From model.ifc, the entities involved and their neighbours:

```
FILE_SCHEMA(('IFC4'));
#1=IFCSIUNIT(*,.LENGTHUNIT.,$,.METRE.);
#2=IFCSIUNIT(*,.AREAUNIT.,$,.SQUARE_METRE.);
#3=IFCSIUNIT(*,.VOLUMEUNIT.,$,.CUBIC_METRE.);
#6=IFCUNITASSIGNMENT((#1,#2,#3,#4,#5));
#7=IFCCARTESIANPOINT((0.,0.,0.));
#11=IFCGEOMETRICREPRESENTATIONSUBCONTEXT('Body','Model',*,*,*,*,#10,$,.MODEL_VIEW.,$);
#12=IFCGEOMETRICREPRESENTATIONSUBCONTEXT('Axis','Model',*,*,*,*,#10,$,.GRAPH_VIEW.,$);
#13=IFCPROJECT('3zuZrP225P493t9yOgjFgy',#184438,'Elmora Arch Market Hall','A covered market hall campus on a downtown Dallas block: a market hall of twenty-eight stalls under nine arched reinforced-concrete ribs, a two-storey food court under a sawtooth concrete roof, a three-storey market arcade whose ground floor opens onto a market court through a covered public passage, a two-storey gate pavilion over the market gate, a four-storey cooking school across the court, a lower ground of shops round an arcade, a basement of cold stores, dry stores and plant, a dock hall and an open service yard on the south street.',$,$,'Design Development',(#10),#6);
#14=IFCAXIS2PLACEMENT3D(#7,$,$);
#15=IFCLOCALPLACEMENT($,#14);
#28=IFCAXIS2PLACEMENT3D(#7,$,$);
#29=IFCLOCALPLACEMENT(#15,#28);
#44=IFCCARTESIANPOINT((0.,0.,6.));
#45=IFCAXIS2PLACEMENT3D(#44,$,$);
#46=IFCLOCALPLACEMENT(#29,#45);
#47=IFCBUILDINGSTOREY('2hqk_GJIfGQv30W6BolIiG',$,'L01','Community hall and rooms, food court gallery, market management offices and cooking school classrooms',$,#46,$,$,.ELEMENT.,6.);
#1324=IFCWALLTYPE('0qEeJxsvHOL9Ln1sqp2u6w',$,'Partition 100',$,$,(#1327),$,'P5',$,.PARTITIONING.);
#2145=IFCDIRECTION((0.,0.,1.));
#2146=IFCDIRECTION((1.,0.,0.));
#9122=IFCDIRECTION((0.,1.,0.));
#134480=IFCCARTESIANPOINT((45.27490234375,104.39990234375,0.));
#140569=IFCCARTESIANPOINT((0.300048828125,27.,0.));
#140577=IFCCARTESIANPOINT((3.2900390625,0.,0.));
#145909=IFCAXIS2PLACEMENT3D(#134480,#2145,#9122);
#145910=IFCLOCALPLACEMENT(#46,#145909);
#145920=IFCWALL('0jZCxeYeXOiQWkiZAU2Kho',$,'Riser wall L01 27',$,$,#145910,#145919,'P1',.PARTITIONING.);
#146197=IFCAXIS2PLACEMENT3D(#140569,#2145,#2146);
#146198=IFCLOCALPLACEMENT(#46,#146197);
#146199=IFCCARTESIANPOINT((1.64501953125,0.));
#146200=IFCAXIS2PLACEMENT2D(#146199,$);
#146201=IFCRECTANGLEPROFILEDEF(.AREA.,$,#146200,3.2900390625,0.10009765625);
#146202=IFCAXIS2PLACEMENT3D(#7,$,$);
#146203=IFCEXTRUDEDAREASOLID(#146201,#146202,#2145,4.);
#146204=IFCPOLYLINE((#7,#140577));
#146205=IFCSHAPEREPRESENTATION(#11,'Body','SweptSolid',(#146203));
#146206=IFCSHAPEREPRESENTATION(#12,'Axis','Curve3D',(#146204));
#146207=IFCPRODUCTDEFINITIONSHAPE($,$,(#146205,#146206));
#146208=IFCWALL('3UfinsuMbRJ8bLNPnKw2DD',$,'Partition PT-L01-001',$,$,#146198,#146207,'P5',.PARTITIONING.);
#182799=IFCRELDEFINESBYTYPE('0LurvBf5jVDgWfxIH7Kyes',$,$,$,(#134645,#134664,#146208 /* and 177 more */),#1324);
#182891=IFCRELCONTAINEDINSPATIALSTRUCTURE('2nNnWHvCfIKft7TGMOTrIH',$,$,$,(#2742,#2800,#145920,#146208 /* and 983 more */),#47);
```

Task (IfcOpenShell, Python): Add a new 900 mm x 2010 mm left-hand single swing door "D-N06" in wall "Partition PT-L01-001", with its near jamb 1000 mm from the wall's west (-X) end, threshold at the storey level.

```python
import numpy as np
import ifcopenshell
import ifcopenshell.api.feature
import ifcopenshell.api.geometry
import ifcopenshell.api.root
import ifcopenshell.api.spatial
import ifcopenshell.geom
import ifcopenshell.util.element
import ifcopenshell.util.placement
import ifcopenshell.util.representation
import ifcopenshell.util.shape
import ifcopenshell.util.unit

model = ifcopenshell.open("model.ifc")
unit_scale = ifcopenshell.util.unit.calculate_unit_scale(model)
settings = ifcopenshell.geom.settings()


def volume(element):
    """Net volume in cubic metres, openings subtracted."""
    shape = ifcopenshell.geom.create_shape(settings, element)
    return ifcopenshell.util.shape.get_volume(shape.geometry)


wall = model.by_id(146208)
storey = ifcopenshell.util.element.get_container(wall, ifc_class="IfcBuildingStorey")
context = ifcopenshell.util.representation.get_context(model, "Model", "Body", "MODEL_VIEW")
before = volume(wall)

width, height, from_end, sill = 0.9, 2.01, 1, 0.0  # metres

# The wall runs along its own X axis, and the end named is its -X end.
wall_shape = ifcopenshell.geom.create_shape(settings, wall)
x, y, z = ifcopenshell.util.shape.get_vertices(wall_shape.geometry).T
start = x.min() + from_end
face, thickness = float(y.min()), float(y.max() - y.min())
wall_matrix = ifcopenshell.util.placement.get_local_placement(wall.ObjectPlacement)
level = ifcopenshell.util.placement.get_local_placement(storey.ObjectPlacement)[2, 3]


def in_wall(x, y):
    """Placement at x, y metres in the wall's axes, at sill height."""
    matrix = wall_matrix.copy()
    matrix[:, 3] = wall_matrix @ np.array([x / unit_scale, y / unit_scale, 0.0, 1.0])
    matrix[2, 3] = level + sill / unit_scale
    return matrix


# Opening: a box that overshoots both wall faces by 50 mm.
opening = ifcopenshell.api.root.create_entity(model, ifc_class="IfcOpeningElement", predefined_type="OPENING")
box = ifcopenshell.api.geometry.add_wall_representation(
    model, context=context, length=width, height=height, thickness=thickness + 0.1
)
ifcopenshell.api.geometry.assign_representation(model, product=opening, representation=box)
ifcopenshell.api.geometry.edit_object_placement(model, product=opening, matrix=in_wall(start, face - 0.05), is_si=False)
ifcopenshell.api.feature.add_feature(model, feature=opening, element=wall)

door = ifcopenshell.api.root.create_entity(model, ifc_class="IfcDoor", name="D-N06", predefined_type="DOOR")
door.OverallWidth, door.OverallHeight = width / unit_scale, height / unit_scale
door.OperationType = "SINGLE_SWING_LEFT"
body = ifcopenshell.api.geometry.add_door_representation(
    model,
    context=context,
    overall_width=door.OverallWidth,
    overall_height=door.OverallHeight,
    operation_type="SINGLE_SWING_LEFT",
    lining_properties={"LiningDepth": thickness / unit_scale, "ThresholdDepth": thickness / unit_scale},
)
ifcopenshell.api.geometry.assign_representation(model, product=door, representation=body)
ifcopenshell.api.spatial.assign_container(model, products=[door], relating_structure=storey)
ifcopenshell.api.feature.add_filling(model, opening=opening, element=door)

# The lining spans the wall, so the door starts at the wall face.
ifcopenshell.api.geometry.edit_object_placement(model, product=door, matrix=in_wall(start, face), is_si=False)

after = volume(wall)

print(f"wall volume {before:.3f} -> {after:.3f} m3")

model.write("model_v2.ifc")
```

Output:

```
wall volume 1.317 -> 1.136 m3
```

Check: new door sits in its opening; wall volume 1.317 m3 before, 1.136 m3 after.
